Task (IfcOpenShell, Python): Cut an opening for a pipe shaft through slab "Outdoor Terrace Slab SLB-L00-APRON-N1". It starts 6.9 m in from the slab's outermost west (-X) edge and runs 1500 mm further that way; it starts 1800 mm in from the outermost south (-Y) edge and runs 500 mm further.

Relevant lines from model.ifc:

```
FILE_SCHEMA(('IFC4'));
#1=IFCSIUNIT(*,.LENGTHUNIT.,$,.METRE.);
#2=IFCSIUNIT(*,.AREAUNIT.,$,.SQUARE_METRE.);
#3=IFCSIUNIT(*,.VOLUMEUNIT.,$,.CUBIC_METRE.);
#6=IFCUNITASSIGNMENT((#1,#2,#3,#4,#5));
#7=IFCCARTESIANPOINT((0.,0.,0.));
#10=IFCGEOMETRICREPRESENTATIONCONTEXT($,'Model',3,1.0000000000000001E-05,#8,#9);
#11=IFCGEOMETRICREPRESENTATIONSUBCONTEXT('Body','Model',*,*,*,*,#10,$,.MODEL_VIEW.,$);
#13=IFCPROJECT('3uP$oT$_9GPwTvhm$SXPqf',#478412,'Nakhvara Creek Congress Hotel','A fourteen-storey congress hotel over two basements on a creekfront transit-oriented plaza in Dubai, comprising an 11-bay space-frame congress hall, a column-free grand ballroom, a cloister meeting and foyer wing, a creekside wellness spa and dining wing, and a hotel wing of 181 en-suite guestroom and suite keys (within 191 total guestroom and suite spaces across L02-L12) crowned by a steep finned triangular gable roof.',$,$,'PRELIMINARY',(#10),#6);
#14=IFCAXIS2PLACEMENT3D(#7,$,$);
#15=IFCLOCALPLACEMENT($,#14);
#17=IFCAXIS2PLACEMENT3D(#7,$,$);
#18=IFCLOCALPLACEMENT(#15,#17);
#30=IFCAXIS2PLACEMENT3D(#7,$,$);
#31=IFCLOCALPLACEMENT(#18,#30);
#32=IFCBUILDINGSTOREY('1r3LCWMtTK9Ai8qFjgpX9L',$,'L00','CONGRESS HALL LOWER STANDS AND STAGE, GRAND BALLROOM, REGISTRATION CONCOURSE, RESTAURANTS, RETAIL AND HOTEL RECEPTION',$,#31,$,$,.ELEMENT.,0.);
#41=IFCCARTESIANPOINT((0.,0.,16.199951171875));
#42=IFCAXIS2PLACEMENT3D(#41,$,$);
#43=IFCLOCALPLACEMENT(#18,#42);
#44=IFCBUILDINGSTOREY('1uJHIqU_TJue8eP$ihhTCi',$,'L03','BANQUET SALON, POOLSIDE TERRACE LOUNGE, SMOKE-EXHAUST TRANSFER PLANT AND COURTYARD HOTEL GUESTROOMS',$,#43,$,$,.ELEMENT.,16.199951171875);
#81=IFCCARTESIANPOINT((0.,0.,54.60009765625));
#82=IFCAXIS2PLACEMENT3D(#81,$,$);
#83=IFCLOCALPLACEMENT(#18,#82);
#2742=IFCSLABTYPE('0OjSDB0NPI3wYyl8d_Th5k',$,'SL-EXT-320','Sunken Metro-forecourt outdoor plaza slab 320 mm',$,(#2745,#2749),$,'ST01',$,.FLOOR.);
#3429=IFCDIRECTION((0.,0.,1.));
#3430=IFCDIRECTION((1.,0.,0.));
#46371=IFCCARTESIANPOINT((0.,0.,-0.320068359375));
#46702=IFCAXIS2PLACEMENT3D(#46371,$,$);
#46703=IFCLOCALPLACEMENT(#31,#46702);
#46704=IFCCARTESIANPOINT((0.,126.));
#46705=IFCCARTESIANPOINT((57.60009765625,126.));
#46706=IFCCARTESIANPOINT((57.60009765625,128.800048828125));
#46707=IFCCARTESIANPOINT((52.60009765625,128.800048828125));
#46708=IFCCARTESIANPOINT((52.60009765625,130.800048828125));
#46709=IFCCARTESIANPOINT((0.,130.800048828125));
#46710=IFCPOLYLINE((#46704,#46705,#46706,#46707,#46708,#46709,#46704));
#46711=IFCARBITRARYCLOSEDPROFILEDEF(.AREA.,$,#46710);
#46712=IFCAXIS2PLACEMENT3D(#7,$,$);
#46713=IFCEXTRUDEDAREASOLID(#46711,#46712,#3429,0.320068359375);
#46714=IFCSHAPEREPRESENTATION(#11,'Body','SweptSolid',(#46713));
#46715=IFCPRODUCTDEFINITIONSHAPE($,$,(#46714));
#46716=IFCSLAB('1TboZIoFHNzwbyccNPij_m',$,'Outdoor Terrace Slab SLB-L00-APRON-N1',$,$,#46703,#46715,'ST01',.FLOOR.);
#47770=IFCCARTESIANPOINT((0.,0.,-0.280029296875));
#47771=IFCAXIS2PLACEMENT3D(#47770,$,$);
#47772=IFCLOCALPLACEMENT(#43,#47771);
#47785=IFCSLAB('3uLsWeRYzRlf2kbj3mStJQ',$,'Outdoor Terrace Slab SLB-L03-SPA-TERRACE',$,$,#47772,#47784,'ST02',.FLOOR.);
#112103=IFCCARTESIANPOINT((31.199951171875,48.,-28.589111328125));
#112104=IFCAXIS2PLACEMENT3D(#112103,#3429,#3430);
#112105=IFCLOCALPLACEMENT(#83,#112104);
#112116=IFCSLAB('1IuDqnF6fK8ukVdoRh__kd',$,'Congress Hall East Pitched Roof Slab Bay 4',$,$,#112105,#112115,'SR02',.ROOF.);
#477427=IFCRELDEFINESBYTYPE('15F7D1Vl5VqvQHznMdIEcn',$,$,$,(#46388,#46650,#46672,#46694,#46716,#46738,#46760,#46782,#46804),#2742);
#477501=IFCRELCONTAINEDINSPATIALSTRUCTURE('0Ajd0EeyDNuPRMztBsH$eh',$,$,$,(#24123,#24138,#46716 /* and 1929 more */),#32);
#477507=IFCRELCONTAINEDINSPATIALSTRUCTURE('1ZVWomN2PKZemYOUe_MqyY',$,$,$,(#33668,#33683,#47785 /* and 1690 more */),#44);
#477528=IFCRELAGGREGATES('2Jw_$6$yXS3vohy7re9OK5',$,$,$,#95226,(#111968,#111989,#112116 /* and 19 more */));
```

```python
import numpy as np
import ifcopenshell
import ifcopenshell.api.feature
import ifcopenshell.api.geometry
import ifcopenshell.api.root
import ifcopenshell.geom
import ifcopenshell.util.placement
import ifcopenshell.util.representation
import ifcopenshell.util.shape
import ifcopenshell.util.unit

model = ifcopenshell.open("model.ifc")
unit_scale = ifcopenshell.util.unit.calculate_unit_scale(model)
settings = ifcopenshell.geom.settings()


def volume(element):
    """Net volume in cubic metres, openings subtracted."""
    shape = ifcopenshell.geom.create_shape(settings, element)
    return ifcopenshell.util.shape.get_volume(shape.geometry)


slab = model.by_id(46716)
before = volume(slab)

# Extent in the slab's own axes, in metres. The edges named are its -X and -Y sides.
slab_shape = ifcopenshell.geom.create_shape(settings, slab)
vertices = ifcopenshell.util.shape.get_vertices(slab_shape.geometry)
x_min, y_min, bottom = vertices.min(axis=0)
top = vertices[:, 2].max()

opening = ifcopenshell.api.root.create_entity(model, ifc_class="IfcOpeningElement", name="Pipe shaft opening", predefined_type="OPENING")
context = ifcopenshell.util.representation.get_context(model, "Model", "Body", "MODEL_VIEW")
width, depth = 1.5, 0.5
outline = [(0.0, 0.0), (width, 0.0), (width, depth), (0.0, depth), (0.0, 0.0)]
# Overshoot both faces by 50 mm so the cut is clean.
shape = ifcopenshell.api.geometry.add_slab_representation(
    model, context=context, depth=top - bottom + 0.1, polyline=outline
)
ifcopenshell.api.geometry.assign_representation(model, product=opening, representation=shape)

matrix = ifcopenshell.util.placement.get_local_placement(slab.ObjectPlacement)
matrix[:, 3] = matrix @ np.append(np.array([x_min + 6.9, y_min + 1.8, bottom - 0.05]) / unit_scale, 1.0)
ifcopenshell.api.geometry.edit_object_placement(model, product=opening, matrix=matrix, is_si=False)
ifcopenshell.api.feature.add_feature(model, feature=opening, element=slab)

after = volume(slab)

print(f"slab volume {before:.3f} -> {after:.3f} m3")

model.write("model-out.ifc")
```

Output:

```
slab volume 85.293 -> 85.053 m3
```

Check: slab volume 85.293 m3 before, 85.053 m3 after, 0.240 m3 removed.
